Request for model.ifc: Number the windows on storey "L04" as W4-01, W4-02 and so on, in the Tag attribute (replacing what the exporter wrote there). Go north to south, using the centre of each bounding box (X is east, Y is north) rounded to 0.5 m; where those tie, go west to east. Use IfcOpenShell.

First a look at what the model holds.

```python
import ifcopenshell
import ifcopenshell.util.element
import ifcopenshell.util.placement

model = ifcopenshell.open("model.ifc")
print(model.schema)
storey = next(s for s in model.by_type("IfcBuildingStorey") if s.Name == "L04")
windows = [e for e in ifcopenshell.util.element.get_decomposition(storey) if e.is_a("IfcWindow")]
for e in sorted(windows, key=lambda e: e.id()):
    origin = ifcopenshell.util.placement.get_local_placement(e.ObjectPlacement)[:3, 3]
    print(e.id(), e.Tag, e.Name, origin.round(2) + 0.0, sep=" | ")
```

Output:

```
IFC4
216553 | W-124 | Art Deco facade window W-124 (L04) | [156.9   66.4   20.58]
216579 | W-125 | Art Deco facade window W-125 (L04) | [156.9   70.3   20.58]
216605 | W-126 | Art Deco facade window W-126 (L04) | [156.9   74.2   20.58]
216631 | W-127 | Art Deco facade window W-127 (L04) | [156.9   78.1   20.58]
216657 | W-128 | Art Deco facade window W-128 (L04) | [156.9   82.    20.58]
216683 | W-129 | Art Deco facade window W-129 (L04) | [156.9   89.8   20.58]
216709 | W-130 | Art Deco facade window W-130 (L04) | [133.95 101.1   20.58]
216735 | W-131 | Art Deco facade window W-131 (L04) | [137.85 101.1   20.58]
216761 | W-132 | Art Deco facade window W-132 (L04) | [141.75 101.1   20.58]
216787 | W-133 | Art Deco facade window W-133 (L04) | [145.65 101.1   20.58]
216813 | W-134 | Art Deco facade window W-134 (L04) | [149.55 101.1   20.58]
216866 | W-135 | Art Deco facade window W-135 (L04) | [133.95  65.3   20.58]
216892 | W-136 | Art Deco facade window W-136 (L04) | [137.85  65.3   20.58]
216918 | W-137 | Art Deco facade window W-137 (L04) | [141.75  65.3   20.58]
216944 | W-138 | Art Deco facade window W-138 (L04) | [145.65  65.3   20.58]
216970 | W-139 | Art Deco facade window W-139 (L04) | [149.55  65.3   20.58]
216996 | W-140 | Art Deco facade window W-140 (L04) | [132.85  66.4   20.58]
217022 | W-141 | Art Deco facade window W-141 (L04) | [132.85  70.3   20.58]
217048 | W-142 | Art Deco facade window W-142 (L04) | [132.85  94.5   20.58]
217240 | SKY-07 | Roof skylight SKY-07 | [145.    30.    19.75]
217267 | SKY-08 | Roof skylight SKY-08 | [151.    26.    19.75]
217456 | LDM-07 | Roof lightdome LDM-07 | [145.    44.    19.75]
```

```python
import ifcopenshell
import ifcopenshell.geom
import ifcopenshell.util.element
import ifcopenshell.util.shape

model = ifcopenshell.open("model.ifc")
settings = ifcopenshell.geom.settings()
settings.set("use-world-coords", True)


def centre(element):
    shape = ifcopenshell.geom.create_shape(settings, element)
    return ifcopenshell.util.shape.get_bbox_centroid(shape.geometry)


storey = next(s for s in model.by_type("IfcBuildingStorey") if s.Name == "L04")
windows = [e for e in ifcopenshell.util.element.get_decomposition(storey) if e.is_a("IfcWindow")]

# Insertion points can sit at a corner or the storey origin, so sort by the geometry (in metres).
centres = {e: centre(e) for e in windows}
windows.sort(key=lambda e: (-round(centres[e][1] / 0.5), centres[e][0]))

for i, e in enumerate(windows, start=1):
    number = f"W4-{i:02d}"
    e.Tag = number
    print(e.id(), number)

model.write("model_rev.ifc")
```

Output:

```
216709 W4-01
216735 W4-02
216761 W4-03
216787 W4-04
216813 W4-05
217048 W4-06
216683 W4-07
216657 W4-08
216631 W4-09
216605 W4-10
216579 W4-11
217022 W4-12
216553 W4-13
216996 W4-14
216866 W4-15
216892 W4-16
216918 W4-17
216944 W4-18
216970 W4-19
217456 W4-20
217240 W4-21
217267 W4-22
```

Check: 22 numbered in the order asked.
